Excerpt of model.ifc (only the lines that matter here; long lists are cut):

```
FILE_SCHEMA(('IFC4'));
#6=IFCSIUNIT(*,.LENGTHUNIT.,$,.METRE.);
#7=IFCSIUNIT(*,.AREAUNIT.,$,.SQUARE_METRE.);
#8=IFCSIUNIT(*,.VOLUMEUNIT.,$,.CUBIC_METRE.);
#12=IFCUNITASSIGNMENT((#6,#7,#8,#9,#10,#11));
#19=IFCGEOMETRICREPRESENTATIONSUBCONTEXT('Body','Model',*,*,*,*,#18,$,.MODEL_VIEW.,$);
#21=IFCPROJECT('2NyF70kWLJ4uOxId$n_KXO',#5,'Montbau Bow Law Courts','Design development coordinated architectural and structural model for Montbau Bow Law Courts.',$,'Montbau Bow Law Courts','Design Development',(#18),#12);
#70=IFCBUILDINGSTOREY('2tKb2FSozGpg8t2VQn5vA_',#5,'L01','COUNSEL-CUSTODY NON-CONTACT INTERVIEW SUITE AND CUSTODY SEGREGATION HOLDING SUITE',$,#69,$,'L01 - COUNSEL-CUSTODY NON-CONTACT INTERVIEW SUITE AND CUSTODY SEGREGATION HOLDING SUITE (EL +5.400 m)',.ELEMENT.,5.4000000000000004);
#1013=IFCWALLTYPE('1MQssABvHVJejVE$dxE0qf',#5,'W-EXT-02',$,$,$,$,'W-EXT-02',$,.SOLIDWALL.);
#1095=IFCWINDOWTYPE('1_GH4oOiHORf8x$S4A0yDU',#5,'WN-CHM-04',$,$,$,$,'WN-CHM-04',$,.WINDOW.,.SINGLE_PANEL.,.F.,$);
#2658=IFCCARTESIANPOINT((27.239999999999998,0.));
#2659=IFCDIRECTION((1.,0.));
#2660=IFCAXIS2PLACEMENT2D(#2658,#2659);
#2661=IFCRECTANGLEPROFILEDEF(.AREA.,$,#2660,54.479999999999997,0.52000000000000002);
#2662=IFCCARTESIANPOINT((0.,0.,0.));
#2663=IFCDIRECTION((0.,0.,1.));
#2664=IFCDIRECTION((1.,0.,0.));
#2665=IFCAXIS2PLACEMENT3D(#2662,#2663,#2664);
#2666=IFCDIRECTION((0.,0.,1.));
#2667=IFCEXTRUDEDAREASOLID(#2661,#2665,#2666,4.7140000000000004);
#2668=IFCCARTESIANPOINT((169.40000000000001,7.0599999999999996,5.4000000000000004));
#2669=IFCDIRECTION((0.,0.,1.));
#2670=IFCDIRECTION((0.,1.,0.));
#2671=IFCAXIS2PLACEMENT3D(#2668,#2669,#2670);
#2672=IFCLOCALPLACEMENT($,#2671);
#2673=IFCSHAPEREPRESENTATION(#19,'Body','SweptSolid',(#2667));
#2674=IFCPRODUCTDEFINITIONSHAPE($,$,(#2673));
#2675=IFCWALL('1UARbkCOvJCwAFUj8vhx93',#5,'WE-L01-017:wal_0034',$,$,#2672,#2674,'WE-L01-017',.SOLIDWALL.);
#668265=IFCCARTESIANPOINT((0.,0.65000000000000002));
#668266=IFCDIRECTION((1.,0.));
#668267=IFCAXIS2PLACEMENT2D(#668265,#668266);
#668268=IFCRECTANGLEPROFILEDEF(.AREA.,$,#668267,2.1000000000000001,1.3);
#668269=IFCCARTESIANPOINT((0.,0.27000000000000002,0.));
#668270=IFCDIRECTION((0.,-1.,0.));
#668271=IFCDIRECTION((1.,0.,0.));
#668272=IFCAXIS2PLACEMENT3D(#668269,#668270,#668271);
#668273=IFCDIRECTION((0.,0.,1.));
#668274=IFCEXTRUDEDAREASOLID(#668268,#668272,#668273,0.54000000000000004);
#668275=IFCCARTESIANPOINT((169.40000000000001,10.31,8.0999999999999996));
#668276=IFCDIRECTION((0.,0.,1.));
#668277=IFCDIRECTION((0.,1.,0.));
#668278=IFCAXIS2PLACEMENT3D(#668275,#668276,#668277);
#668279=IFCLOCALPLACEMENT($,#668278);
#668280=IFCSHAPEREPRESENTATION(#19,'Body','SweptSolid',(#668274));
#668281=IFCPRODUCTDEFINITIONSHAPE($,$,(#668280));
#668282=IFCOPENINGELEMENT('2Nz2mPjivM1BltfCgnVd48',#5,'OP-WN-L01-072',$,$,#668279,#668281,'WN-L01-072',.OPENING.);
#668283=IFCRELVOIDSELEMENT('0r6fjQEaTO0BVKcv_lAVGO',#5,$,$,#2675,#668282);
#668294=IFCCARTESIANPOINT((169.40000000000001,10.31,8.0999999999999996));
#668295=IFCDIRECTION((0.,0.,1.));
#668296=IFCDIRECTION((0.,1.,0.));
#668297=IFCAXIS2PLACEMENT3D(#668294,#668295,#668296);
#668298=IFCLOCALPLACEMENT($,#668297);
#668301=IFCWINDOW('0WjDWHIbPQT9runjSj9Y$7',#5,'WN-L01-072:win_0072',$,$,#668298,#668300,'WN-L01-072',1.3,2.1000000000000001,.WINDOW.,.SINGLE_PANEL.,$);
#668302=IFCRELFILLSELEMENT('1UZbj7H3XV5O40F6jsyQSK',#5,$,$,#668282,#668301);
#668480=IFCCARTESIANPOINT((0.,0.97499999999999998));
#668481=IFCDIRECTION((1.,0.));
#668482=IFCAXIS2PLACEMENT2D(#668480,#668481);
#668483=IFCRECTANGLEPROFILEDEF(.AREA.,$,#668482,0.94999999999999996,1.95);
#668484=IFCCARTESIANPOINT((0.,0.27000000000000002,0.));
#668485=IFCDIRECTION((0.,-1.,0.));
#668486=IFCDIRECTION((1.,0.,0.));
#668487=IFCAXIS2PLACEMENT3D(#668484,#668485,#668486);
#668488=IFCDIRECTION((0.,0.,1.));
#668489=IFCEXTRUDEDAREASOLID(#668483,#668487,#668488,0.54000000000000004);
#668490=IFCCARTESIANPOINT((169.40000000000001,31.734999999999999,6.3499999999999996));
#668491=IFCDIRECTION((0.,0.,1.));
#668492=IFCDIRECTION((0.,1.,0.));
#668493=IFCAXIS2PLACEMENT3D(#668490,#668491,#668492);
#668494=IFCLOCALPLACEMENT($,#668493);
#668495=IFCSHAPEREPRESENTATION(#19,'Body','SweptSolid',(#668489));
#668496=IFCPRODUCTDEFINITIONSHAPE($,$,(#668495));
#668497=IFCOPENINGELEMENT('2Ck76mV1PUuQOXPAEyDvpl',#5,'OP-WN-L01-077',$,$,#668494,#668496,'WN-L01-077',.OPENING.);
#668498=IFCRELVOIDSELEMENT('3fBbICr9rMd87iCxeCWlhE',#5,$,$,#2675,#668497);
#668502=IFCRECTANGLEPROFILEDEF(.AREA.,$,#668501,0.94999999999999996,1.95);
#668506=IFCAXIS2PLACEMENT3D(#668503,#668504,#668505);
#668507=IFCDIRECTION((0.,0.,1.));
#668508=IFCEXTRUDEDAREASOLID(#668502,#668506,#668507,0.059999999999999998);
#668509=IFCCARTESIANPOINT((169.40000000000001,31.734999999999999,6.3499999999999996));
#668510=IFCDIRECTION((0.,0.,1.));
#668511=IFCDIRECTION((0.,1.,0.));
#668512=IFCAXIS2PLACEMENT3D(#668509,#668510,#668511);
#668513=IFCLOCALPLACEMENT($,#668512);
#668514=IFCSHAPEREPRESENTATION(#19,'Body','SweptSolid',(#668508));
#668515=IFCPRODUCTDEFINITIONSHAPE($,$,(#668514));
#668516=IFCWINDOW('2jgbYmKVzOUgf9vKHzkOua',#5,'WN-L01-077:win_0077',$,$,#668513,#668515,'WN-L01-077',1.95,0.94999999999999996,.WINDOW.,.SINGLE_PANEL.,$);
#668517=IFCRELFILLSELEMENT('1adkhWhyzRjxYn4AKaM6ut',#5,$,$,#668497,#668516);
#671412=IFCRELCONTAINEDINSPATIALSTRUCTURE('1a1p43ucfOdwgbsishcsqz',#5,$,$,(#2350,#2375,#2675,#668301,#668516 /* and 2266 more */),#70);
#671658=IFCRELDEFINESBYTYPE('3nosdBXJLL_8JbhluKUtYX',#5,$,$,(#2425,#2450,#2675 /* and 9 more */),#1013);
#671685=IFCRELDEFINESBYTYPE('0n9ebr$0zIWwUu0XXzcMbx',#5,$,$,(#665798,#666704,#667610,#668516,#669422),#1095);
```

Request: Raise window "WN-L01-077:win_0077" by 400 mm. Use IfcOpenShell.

```python
import numpy as np
import ifcopenshell
import ifcopenshell.api.geometry
import ifcopenshell.util.placement
import ifcopenshell.util.unit

model = ifcopenshell.open("model.ifc")
unit_scale = ifcopenshell.util.unit.calculate_unit_scale(model)

window = model.by_guid("2jgbYmKVzOUgf9vKHzkOua")
opening = window.FillsVoids[0].RelatingOpeningElement
dz = 0.4 / unit_scale

shift = np.array([0.0, 0.0, dz])
# The window is not placed relative to its opening, so move both.
for product in (opening, window):
    matrix = ifcopenshell.util.placement.get_local_placement(product.ObjectPlacement)
    matrix[:3, 3] += shift
    ifcopenshell.api.geometry.edit_object_placement(model, product=product, matrix=matrix, is_si=False)

print(f"moved by {dz * unit_scale:+.3f} m")

model.write("model_rev.ifc")
```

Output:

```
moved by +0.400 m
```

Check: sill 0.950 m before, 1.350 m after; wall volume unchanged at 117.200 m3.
